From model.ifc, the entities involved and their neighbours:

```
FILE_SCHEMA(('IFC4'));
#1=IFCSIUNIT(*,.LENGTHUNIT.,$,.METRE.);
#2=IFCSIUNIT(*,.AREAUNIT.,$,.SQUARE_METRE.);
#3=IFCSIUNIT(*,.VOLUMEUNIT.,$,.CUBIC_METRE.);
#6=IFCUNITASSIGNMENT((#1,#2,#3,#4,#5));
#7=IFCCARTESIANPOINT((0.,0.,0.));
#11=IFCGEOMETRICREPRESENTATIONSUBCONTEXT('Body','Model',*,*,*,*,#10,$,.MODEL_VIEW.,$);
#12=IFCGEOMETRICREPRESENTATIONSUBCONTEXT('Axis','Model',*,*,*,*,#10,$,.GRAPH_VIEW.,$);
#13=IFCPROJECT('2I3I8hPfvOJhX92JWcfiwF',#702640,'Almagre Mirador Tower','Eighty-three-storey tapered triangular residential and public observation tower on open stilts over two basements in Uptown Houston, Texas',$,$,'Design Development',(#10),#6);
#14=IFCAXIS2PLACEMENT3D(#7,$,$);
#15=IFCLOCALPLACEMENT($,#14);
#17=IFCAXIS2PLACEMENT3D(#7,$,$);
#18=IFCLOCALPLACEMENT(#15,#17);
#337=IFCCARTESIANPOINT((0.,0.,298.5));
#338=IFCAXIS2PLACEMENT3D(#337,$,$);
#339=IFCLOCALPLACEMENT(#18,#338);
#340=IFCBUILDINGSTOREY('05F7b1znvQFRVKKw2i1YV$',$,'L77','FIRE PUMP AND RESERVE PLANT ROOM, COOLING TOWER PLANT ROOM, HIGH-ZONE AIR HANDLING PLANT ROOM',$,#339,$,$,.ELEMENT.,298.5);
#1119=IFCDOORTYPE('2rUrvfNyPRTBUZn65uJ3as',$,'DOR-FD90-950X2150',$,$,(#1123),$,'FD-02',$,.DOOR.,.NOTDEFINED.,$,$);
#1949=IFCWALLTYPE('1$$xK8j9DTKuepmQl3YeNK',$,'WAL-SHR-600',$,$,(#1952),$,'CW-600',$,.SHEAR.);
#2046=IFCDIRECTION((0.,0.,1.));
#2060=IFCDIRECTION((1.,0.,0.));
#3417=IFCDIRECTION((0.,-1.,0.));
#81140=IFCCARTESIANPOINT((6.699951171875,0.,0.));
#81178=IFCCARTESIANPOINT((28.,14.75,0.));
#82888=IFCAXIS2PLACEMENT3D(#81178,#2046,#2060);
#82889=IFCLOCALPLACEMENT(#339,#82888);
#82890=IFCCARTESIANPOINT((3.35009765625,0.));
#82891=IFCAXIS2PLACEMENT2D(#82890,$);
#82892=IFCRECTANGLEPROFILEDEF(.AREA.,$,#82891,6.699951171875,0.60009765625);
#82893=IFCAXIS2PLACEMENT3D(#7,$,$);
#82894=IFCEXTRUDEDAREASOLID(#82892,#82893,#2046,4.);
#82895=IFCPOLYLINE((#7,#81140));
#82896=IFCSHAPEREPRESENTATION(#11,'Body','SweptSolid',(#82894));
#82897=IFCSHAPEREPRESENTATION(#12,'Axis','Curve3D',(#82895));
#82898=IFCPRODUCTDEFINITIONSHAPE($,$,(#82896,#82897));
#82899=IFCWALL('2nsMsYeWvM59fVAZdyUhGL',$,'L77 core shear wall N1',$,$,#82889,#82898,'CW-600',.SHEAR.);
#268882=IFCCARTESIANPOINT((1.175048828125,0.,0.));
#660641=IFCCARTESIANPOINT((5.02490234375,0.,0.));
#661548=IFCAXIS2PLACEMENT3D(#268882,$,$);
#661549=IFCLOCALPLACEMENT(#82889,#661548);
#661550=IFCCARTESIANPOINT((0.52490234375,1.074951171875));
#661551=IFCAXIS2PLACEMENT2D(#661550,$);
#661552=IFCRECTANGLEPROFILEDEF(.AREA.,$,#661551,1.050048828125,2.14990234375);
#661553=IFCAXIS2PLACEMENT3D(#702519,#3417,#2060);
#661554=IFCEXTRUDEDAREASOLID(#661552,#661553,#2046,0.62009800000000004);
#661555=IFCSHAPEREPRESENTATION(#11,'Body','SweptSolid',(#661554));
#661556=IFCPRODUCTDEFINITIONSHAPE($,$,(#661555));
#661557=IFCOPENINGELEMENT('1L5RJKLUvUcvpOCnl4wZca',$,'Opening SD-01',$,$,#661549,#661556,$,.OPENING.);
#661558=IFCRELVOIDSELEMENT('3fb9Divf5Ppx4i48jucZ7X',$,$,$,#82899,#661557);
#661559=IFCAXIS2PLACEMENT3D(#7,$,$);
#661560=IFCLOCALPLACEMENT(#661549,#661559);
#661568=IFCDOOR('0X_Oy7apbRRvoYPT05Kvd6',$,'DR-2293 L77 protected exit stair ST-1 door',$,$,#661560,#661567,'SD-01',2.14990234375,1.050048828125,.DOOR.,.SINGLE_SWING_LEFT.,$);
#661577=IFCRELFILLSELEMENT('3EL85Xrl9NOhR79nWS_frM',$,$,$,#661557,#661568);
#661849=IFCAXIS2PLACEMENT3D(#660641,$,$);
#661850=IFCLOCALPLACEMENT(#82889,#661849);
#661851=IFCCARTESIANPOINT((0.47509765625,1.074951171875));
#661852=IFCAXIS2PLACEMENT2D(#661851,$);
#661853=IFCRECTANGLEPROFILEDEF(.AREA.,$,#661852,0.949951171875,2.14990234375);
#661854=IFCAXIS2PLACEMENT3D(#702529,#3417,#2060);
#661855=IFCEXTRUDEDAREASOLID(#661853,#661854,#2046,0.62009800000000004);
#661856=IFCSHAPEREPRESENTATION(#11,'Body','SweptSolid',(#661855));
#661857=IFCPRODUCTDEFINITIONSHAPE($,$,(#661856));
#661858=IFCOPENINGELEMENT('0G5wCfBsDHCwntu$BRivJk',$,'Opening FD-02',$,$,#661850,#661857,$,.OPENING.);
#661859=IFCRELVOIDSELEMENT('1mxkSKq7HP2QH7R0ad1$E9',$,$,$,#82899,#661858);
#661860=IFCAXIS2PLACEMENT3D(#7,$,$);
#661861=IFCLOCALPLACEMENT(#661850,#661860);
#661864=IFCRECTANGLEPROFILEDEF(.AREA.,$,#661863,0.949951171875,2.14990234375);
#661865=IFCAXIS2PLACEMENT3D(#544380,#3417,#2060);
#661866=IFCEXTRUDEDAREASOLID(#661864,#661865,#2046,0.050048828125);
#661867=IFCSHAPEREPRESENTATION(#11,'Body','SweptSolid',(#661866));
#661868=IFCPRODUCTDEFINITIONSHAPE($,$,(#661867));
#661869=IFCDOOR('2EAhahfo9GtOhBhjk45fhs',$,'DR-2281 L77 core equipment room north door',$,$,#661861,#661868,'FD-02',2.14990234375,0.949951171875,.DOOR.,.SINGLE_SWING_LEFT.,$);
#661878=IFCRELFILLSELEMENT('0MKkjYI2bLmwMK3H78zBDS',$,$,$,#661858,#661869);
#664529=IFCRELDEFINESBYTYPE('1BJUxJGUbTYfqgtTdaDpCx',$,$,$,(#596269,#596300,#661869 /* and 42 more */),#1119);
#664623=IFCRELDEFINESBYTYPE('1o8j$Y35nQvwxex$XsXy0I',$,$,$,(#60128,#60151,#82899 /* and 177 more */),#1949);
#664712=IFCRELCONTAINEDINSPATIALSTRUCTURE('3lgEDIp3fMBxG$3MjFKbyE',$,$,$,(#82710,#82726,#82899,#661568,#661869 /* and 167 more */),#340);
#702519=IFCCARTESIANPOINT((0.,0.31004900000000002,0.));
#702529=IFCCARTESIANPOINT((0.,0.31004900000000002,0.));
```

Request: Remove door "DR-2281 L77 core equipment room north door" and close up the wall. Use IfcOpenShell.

```python
import ifcopenshell
import ifcopenshell.api.feature
import ifcopenshell.api.root
import ifcopenshell.geom
import ifcopenshell.util.shape

model = ifcopenshell.open("model.ifc")
settings = ifcopenshell.geom.settings()


def volume(element):
    """Net volume in cubic metres, openings subtracted."""
    shape = ifcopenshell.geom.create_shape(settings, element)
    return ifcopenshell.util.shape.get_volume(shape.geometry)


door = model.by_id(661869)
opening = door.FillsVoids[0].RelatingOpeningElement
wall = opening.VoidsElements[0].RelatingBuildingElement
before = volume(wall)

ifcopenshell.api.root.remove_product(model, product=door)
ifcopenshell.api.feature.remove_feature(model, feature=opening)

after = volume(wall)

print(f"wall volume {before:.3f} -> {after:.3f} m3")

model.write("model_updated.ifc")
```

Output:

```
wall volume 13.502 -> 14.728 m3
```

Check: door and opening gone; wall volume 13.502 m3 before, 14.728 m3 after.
